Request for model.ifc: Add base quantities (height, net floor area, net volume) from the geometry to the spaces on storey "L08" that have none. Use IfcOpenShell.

First a look at what the model holds.

```python
import ifcopenshell
import ifcopenshell.util.element
import ifcopenshell.util.unit

model = ifcopenshell.open("model.ifc")
print(model.schema)
for unit_type in ("LENGTHUNIT", "AREAUNIT", "VOLUMEUNIT"):
    print(unit_type, ifcopenshell.util.unit.calculate_unit_scale(model, unit_type))
storey = next(s for s in model.by_type("IfcBuildingStorey") if s.Name == "L08")
spaces = [e for e in ifcopenshell.util.element.get_decomposition(storey) if e.is_a("IfcSpace")]
for e in sorted(spaces, key=lambda e: e.id()):
    print(e.id(), e.is_a(), e.Name, list(ifcopenshell.util.element.get_psets(e, qtos_only=True)), sep=" | ")
```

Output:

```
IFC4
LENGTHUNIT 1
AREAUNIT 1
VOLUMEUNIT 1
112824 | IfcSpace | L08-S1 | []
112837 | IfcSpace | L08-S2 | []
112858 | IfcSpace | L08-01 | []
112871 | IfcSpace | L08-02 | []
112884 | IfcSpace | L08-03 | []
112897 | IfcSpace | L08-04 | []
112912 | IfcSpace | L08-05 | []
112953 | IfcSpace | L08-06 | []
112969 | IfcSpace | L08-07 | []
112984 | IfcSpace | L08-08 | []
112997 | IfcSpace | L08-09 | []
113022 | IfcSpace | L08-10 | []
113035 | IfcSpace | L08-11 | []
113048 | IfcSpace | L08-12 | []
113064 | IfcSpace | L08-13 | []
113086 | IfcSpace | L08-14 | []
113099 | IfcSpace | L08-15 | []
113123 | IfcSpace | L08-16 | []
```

```python
import ifcopenshell
import ifcopenshell.api.pset
import ifcopenshell.geom
import ifcopenshell.util.element
import ifcopenshell.util.shape
import ifcopenshell.util.unit

model = ifcopenshell.open("model.ifc")
unit_scale = ifcopenshell.util.unit.calculate_unit_scale(model)
area_scale = ifcopenshell.util.unit.calculate_unit_scale(model, "AREAUNIT")
volume_scale = ifcopenshell.util.unit.calculate_unit_scale(model, "VOLUMEUNIT")
settings = ifcopenshell.geom.settings()

storey = next(s for s in model.by_type("IfcBuildingStorey") if s.Name == "L08")
spaces = [e for e in ifcopenshell.util.element.get_decomposition(storey) if e.is_a("IfcSpace")]

for e in sorted(spaces, key=lambda e: e.id()):
    if ifcopenshell.util.element.get_psets(e, qtos_only=True, should_inherit=False):
        continue
    # Geometry comes back in metres, in the element's own axes.
    shape = ifcopenshell.geom.create_shape(settings, e)
    values = {
        "Height": ifcopenshell.util.shape.get_z(shape.geometry) / unit_scale,
        "NetFloorArea": ifcopenshell.util.shape.get_footprint_area(shape.geometry) / area_scale,
        "NetVolume": ifcopenshell.util.shape.get_volume(shape.geometry) / volume_scale,
    }
    qto = ifcopenshell.api.pset.add_qto(model, product=e, name="Qto_SpaceBaseQuantities")
    ifcopenshell.api.pset.edit_qto(model, qto=qto, properties=values)
    print(e.id(), {k: round(v, 3) for k, v in values.items()})

model.write("model-out.ifc")
```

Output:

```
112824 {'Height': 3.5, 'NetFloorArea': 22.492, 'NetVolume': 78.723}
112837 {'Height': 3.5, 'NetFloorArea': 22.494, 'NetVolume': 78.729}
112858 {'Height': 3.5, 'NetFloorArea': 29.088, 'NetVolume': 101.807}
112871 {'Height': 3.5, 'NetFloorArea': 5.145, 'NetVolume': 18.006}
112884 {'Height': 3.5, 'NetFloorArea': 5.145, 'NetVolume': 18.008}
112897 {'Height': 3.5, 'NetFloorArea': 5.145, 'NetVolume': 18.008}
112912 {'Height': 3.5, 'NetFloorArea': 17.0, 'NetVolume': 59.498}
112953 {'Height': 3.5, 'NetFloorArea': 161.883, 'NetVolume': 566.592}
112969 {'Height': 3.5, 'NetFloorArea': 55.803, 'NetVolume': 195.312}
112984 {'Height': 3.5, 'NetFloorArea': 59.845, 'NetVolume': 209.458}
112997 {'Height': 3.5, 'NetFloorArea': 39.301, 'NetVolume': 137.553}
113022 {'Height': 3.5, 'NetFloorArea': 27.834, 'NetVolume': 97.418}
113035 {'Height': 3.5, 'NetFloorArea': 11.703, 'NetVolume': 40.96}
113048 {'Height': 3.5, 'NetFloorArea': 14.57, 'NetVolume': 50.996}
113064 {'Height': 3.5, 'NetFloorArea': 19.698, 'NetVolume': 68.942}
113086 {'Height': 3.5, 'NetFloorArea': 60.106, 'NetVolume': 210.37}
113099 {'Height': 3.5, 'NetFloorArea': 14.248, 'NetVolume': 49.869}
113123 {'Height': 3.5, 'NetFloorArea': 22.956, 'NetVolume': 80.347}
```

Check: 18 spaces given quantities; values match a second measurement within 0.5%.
